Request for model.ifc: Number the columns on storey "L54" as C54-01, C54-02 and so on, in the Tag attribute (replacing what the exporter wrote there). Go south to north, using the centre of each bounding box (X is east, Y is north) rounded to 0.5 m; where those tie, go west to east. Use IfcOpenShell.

First a look at what the model holds.

```python
import ifcopenshell
import ifcopenshell.util.element
import ifcopenshell.util.placement

model = ifcopenshell.open("model.ifc")
print(model.schema)
storey = next(s for s in model.by_type("IfcBuildingStorey") if s.Name == "L54")
columns = [e for e in ifcopenshell.util.element.get_decomposition(storey) if e.is_a("IfcColumn")]
for e in sorted(columns, key=lambda e: e.id()):
    origin = ifcopenshell.util.placement.get_local_placement(e.ObjectPlacement)[:3, 3]
    print(e.id(), e.Tag, e.Name, origin.round(2) + 0.0, sep=" | ")
```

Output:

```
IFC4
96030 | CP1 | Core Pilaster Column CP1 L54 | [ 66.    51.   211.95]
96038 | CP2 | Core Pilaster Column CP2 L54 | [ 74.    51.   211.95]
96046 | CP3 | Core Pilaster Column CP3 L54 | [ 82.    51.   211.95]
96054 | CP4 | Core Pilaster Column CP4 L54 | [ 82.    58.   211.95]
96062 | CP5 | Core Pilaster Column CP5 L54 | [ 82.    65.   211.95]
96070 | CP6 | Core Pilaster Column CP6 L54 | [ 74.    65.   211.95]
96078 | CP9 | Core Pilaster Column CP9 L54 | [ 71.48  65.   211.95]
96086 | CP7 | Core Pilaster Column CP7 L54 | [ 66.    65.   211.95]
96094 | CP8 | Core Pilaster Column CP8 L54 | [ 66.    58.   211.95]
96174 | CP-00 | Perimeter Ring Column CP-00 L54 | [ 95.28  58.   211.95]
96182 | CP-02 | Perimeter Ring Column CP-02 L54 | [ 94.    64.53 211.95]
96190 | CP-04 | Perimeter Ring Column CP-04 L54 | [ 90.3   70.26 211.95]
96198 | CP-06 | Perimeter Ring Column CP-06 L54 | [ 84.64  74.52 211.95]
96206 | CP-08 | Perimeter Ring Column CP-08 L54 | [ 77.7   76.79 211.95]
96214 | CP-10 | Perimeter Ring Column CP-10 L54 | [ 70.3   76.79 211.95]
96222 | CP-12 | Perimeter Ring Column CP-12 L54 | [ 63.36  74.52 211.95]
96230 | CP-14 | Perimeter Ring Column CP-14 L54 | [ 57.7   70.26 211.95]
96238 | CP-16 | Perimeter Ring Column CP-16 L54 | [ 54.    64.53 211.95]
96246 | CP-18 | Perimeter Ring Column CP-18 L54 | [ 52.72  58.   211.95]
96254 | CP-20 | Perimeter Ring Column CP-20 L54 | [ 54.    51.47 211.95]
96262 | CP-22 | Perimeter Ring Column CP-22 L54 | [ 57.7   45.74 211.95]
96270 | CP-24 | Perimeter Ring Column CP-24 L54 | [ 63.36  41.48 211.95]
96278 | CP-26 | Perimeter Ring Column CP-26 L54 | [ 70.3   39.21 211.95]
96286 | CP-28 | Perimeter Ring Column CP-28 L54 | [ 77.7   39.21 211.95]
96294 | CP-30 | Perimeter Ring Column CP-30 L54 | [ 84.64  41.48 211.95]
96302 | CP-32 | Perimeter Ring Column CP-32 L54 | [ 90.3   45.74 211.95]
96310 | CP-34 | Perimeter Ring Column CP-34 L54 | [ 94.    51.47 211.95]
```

```python
import ifcopenshell
import ifcopenshell.geom
import ifcopenshell.util.element
import ifcopenshell.util.shape

model = ifcopenshell.open("model.ifc")
settings = ifcopenshell.geom.settings()
settings.set("use-world-coords", True)


def centre(element):
    shape = ifcopenshell.geom.create_shape(settings, element)
    return ifcopenshell.util.shape.get_bbox_centroid(shape.geometry)


storey = next(s for s in model.by_type("IfcBuildingStorey") if s.Name == "L54")
columns = [e for e in ifcopenshell.util.element.get_decomposition(storey) if e.is_a("IfcColumn")]

# Insertion points can sit at a corner or the storey origin, so sort by the geometry (in metres).
centres = {e: centre(e) for e in columns}
columns.sort(key=lambda e: (round(centres[e][1] / 0.5), centres[e][0]))

for i, e in enumerate(columns, start=1):
    number = f"C54-{i:02d}"
    e.Tag = number
    print(e.id(), number)

model.write("model_edited.ifc")
```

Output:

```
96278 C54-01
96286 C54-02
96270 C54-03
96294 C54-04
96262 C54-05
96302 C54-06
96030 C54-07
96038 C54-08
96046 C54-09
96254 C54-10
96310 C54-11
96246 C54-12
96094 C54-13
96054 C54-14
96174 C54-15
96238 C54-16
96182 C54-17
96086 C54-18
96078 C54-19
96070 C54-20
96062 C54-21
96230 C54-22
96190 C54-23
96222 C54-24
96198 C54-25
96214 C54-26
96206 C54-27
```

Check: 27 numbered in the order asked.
